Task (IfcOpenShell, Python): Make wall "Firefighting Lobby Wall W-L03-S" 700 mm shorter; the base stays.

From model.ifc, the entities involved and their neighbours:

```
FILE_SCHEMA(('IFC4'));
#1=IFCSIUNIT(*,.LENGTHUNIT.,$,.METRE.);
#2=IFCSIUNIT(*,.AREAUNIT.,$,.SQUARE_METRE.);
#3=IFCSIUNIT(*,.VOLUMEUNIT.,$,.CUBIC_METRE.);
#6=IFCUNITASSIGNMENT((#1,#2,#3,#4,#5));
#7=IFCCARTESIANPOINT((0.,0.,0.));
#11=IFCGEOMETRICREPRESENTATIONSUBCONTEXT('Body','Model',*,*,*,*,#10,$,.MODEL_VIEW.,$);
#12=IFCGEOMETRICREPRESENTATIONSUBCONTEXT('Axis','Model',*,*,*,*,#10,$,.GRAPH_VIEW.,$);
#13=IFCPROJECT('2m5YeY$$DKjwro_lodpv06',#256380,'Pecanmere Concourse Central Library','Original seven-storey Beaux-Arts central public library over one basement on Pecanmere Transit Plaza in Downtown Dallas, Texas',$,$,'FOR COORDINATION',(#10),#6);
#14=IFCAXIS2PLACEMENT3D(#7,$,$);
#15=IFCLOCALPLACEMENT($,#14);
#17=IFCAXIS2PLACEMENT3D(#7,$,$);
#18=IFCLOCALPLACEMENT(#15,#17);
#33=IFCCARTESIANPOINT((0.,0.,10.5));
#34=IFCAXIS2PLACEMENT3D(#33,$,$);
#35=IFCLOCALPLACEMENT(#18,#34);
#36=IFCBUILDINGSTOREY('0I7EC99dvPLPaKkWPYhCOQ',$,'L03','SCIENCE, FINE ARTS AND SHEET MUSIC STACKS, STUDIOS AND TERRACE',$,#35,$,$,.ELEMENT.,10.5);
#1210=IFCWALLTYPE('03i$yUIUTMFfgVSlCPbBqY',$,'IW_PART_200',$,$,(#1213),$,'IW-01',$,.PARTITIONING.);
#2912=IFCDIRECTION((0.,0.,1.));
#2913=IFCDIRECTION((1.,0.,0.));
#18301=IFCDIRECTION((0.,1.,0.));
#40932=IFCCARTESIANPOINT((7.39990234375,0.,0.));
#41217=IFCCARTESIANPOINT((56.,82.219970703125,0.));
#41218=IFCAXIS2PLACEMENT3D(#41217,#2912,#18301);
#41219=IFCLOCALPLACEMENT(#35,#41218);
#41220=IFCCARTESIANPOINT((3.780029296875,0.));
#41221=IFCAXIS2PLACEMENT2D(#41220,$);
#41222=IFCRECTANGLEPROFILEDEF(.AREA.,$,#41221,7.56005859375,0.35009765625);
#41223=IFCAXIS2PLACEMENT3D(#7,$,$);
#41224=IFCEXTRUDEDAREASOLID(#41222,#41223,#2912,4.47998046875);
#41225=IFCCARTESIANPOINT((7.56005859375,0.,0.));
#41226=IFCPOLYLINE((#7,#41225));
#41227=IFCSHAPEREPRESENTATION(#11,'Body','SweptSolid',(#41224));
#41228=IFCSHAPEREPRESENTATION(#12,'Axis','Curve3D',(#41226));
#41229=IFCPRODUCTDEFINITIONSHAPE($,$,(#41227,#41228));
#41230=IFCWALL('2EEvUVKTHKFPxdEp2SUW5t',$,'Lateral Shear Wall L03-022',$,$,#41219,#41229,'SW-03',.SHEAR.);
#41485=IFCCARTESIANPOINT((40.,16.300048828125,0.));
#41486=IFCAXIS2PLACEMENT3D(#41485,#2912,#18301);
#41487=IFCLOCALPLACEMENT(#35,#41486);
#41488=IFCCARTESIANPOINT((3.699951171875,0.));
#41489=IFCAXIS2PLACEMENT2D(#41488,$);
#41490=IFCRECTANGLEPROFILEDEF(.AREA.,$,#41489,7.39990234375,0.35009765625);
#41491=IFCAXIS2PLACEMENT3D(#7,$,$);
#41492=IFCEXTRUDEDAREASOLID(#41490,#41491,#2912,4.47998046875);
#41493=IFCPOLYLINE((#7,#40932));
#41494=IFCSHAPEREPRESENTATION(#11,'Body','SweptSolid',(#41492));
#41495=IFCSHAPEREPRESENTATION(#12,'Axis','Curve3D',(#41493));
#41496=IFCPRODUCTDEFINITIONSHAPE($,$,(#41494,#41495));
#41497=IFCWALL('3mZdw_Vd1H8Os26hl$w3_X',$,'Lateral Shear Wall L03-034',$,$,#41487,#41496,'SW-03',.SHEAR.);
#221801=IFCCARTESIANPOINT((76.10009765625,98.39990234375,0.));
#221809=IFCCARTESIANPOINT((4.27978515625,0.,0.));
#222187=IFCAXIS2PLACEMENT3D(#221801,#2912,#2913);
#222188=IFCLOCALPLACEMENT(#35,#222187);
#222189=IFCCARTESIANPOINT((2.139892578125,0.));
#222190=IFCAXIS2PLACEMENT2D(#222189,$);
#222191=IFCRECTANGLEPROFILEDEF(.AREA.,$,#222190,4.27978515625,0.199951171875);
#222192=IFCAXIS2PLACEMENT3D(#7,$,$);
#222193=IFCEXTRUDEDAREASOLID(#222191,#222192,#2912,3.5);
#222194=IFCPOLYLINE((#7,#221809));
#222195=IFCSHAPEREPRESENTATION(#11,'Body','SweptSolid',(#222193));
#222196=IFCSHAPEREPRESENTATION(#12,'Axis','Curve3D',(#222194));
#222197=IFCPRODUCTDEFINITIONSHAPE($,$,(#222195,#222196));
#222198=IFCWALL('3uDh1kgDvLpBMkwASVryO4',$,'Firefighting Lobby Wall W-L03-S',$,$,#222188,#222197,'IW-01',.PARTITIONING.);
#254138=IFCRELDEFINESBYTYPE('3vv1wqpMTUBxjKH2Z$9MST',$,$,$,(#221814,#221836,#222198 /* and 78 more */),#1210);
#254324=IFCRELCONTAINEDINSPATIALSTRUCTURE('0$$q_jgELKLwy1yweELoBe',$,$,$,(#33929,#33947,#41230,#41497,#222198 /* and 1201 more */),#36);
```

```python
import ifcopenshell
import ifcopenshell.geom
import ifcopenshell.util.representation
import ifcopenshell.util.shape
import ifcopenshell.util.unit

model = ifcopenshell.open("model.ifc")
unit_scale = ifcopenshell.util.unit.calculate_unit_scale(model)
settings = ifcopenshell.geom.settings()


def volume(element):
    """Net volume in cubic metres, openings subtracted."""
    shape = ifcopenshell.geom.create_shape(settings, element)
    return ifcopenshell.util.shape.get_volume(shape.geometry)


wall = model.by_guid("3uDh1kgDvLpBMkwASVryO4")
before = volume(wall)

body = ifcopenshell.util.representation.get_representation(wall, "Model", "Body")
solid = body.Items[0]
old_height = solid.Depth
solid.Depth -= 0.7 / unit_scale
after = volume(wall)

print(f"height {old_height:g} -> {solid.Depth:g}, volume {before:.3f} -> {after:.3f} m3")

model.write("model-out.ifc")
```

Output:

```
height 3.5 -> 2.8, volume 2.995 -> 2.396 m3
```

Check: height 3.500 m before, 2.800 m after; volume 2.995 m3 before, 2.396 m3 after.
